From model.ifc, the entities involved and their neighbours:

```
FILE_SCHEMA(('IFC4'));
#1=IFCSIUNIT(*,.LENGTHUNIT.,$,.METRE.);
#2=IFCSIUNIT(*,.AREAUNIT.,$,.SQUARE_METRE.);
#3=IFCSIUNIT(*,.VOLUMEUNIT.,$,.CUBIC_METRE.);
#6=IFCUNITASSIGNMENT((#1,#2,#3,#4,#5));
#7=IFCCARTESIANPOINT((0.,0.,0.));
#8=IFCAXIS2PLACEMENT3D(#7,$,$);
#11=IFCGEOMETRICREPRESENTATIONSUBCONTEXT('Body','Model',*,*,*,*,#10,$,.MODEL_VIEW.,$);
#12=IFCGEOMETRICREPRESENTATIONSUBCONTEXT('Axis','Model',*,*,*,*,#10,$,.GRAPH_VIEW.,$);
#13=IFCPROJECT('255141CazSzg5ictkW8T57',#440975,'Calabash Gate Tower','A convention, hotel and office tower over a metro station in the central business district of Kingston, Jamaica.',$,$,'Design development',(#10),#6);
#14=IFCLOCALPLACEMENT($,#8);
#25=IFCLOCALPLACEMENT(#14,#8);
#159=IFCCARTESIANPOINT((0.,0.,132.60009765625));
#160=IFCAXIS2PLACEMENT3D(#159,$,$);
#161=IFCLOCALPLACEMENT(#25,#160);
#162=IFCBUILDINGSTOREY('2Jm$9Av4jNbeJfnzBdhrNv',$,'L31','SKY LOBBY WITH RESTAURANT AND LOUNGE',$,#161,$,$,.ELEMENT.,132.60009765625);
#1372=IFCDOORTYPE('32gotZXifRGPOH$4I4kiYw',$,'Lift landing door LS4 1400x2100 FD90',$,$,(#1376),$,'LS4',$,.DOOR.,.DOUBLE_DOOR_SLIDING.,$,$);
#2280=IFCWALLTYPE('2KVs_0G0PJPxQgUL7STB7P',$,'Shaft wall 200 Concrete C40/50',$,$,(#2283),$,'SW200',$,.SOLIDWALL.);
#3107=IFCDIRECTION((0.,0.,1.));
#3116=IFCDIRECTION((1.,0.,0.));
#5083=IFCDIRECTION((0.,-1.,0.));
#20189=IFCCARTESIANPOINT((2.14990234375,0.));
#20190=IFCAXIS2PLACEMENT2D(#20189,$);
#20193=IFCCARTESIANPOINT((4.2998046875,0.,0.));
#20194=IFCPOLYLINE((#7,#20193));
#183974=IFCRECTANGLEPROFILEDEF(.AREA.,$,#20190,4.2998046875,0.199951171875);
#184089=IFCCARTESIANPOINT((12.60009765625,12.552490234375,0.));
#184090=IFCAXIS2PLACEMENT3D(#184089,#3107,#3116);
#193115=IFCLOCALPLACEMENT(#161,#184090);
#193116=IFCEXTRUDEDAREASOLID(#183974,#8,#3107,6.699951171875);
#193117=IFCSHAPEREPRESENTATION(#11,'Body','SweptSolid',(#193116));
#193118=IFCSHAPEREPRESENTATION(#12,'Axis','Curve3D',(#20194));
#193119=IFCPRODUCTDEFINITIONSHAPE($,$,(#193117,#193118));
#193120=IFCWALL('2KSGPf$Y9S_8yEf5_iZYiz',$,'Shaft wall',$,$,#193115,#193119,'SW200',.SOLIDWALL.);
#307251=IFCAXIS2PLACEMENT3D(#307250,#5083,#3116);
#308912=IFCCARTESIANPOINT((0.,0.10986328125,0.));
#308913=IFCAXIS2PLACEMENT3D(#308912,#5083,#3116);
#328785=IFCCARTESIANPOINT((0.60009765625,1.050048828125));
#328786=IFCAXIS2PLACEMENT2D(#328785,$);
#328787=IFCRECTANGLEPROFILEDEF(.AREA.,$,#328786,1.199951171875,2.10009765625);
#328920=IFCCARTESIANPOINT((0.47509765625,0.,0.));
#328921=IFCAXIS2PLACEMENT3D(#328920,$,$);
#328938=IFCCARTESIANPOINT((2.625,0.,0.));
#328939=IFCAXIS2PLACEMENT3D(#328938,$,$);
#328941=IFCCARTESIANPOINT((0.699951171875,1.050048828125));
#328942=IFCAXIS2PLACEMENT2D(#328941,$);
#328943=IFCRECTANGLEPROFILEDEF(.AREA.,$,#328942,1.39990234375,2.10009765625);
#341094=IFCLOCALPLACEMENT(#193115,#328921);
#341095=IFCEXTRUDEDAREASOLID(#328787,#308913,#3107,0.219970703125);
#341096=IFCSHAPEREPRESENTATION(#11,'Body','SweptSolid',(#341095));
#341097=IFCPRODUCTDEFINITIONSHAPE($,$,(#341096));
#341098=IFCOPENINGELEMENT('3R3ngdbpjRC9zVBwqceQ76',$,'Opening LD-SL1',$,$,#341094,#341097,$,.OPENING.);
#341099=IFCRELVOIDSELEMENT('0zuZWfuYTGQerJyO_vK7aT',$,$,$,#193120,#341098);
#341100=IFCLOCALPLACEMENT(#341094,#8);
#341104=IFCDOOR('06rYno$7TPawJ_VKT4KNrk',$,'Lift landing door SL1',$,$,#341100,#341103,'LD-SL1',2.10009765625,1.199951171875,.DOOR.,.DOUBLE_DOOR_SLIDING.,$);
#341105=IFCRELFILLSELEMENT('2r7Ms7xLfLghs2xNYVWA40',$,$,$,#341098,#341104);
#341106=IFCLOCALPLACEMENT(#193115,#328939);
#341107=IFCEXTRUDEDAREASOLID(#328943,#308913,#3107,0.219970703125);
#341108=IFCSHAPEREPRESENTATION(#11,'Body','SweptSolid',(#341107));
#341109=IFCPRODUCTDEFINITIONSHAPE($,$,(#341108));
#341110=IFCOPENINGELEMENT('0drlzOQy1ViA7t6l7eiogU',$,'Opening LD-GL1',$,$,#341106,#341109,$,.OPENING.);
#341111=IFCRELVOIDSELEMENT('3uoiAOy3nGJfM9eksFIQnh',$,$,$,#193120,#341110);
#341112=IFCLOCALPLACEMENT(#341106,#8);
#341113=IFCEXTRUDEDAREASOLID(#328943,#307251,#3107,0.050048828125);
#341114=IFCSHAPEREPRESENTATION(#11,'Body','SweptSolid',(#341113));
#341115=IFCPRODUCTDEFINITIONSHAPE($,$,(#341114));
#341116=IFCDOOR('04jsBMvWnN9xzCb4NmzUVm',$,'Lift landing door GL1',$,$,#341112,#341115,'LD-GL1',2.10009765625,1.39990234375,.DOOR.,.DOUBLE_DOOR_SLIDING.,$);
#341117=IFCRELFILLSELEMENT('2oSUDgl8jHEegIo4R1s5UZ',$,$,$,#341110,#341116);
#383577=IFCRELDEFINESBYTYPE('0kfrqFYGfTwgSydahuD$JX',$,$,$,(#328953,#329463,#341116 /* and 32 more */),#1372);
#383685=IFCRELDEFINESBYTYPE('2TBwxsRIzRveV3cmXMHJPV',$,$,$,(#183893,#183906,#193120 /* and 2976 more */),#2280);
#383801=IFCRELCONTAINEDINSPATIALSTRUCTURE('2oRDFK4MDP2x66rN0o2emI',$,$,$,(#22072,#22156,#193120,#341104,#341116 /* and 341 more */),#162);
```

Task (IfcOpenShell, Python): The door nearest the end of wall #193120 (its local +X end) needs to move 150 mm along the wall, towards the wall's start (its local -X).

```python
import ifcopenshell
import ifcopenshell.api.geometry
import ifcopenshell.util.placement

model = ifcopenshell.open("model.ifc")

door = model.by_guid("04jsBMvWnN9xzCb4NmzUVm")
opening = door.FillsVoids[0].RelatingOpeningElement
wall = opening.VoidsElements[0].RelatingBuildingElement

wall_matrix = ifcopenshell.util.placement.get_local_placement(wall.ObjectPlacement)
shift = wall_matrix[:3, 0] * -0.15
before = ifcopenshell.util.placement.get_local_placement(door.ObjectPlacement)[:3, 3].copy()

# The door is placed relative to its opening, so it follows when the opening moves.
matrix = ifcopenshell.util.placement.get_local_placement(opening.ObjectPlacement)
matrix[:3, 3] += shift
ifcopenshell.api.geometry.edit_object_placement(
    model, product=opening, matrix=matrix, is_si=False, should_transform_children=True
)

after = ifcopenshell.util.placement.get_local_placement(door.ObjectPlacement)[:3, 3]
print("door moved by", (after - before).round(3) + 0.0)

model.write("model_rev.ifc")
```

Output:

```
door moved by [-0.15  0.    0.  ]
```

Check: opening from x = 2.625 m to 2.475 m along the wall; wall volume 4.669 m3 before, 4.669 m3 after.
